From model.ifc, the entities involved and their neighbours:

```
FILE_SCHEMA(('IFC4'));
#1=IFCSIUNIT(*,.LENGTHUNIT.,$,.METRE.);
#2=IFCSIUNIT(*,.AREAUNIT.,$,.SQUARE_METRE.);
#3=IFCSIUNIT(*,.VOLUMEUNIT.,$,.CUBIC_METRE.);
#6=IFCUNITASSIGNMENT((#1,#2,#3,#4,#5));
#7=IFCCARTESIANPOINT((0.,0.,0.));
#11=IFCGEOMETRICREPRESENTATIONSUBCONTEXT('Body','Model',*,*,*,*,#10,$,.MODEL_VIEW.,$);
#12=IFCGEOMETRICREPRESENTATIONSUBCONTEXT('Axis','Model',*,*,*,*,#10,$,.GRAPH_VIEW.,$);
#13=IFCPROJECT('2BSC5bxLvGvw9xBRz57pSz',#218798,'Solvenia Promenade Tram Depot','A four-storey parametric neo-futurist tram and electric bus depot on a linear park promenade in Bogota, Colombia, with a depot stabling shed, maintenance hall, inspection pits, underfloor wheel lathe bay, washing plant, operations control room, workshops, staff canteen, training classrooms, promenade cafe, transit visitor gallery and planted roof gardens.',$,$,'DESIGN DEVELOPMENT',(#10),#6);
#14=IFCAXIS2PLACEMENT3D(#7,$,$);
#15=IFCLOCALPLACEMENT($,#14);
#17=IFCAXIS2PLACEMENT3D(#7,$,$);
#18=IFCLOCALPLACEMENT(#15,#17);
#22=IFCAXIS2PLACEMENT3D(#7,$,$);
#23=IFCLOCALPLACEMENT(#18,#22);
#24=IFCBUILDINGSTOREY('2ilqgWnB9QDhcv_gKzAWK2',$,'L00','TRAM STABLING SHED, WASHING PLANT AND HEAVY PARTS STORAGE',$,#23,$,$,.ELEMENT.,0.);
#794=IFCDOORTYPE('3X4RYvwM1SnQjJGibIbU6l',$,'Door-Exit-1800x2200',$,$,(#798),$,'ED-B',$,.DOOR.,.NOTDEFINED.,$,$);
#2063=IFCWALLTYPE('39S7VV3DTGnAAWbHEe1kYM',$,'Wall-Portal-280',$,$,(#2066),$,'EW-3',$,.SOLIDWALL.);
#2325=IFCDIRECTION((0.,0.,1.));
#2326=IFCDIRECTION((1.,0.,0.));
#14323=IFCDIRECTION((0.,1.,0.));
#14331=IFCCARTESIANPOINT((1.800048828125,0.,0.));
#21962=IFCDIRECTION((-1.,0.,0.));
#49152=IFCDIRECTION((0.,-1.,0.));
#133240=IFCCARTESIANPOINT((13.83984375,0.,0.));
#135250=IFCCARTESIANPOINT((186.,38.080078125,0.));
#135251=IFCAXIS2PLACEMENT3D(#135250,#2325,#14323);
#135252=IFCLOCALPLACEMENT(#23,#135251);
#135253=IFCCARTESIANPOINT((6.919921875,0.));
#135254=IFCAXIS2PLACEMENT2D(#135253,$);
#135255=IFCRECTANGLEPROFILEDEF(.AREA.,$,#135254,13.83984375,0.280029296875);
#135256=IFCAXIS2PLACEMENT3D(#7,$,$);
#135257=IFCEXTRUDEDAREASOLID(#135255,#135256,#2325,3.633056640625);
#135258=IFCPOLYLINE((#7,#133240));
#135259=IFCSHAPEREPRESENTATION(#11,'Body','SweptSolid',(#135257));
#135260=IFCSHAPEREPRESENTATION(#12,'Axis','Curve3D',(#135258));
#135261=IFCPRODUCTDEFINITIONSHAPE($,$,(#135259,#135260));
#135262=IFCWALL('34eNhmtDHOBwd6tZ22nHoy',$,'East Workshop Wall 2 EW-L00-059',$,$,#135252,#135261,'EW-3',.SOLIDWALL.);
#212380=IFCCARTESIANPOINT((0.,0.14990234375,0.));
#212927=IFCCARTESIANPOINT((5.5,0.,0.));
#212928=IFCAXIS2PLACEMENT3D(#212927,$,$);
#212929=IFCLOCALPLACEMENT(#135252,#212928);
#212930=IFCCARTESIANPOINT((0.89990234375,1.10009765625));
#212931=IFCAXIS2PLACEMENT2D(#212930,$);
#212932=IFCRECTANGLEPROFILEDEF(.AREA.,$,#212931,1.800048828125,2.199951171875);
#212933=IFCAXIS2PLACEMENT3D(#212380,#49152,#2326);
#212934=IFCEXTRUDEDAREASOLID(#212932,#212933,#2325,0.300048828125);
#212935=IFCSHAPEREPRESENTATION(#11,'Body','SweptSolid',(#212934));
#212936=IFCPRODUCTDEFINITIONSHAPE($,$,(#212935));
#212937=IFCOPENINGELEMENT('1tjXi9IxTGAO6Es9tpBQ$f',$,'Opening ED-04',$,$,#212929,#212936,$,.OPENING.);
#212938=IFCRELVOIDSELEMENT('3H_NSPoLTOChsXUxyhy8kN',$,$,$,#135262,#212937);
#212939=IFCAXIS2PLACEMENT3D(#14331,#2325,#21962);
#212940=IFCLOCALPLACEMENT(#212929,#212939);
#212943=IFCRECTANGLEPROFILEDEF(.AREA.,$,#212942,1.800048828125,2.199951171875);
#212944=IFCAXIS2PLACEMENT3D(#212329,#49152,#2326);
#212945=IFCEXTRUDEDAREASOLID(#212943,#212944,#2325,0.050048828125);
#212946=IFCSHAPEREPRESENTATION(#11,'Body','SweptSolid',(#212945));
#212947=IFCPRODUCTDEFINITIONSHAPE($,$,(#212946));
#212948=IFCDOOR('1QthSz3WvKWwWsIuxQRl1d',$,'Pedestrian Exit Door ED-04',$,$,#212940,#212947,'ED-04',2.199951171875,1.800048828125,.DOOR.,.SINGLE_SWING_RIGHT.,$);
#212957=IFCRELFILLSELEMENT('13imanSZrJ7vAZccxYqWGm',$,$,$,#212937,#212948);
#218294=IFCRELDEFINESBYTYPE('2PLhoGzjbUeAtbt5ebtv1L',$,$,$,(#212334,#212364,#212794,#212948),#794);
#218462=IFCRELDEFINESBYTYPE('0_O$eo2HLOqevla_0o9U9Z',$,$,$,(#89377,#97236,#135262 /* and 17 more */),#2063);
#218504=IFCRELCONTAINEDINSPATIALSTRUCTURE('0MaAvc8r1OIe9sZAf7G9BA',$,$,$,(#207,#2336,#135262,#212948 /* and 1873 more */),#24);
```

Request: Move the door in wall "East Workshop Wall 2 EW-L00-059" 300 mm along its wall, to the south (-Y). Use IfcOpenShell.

```python
import ifcopenshell
import ifcopenshell.api.geometry
import ifcopenshell.util.placement

model = ifcopenshell.open("model.ifc")

door = model.by_guid("1QthSz3WvKWwWsIuxQRl1d")
opening = door.FillsVoids[0].RelatingOpeningElement
wall = opening.VoidsElements[0].RelatingBuildingElement

wall_matrix = ifcopenshell.util.placement.get_local_placement(wall.ObjectPlacement)
shift = wall_matrix[:3, 0] * -0.3
before = ifcopenshell.util.placement.get_local_placement(door.ObjectPlacement)[:3, 3].copy()

# The door is placed relative to its opening, so it follows when the opening moves.
matrix = ifcopenshell.util.placement.get_local_placement(opening.ObjectPlacement)
matrix[:3, 3] += shift
ifcopenshell.api.geometry.edit_object_placement(
    model, product=opening, matrix=matrix, is_si=False, should_transform_children=True
)

after = ifcopenshell.util.placement.get_local_placement(door.ObjectPlacement)[:3, 3]
print("door moved by", (after - before).round(3) + 0.0)

model.write("model_v2.ifc")
```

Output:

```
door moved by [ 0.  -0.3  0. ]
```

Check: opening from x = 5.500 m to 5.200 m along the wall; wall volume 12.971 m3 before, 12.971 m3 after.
